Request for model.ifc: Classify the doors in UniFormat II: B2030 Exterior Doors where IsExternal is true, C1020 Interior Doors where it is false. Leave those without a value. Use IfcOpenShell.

First a look at what the model holds.

```python
import ifcopenshell
import ifcopenshell.util.element

model = ifcopenshell.open("model.ifc")
print(model.schema)
print("classifications:", [c.Name for c in model.by_type("IfcClassification")])
values = [ifcopenshell.util.element.get_pset(e, "Pset_DoorCommon", "IsExternal") for e in model.by_type("IfcDoor")]
for value in (True, False, None):
    print("IsExternal", value, values.count(value))
```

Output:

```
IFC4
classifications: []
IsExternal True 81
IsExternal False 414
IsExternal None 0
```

```python
import ifcopenshell
import ifcopenshell.api.classification
import ifcopenshell.util.element

model = ifcopenshell.open("model.ifc")

system = ifcopenshell.api.classification.add_classification(model, classification="UniFormat II")

doors = model.by_type("IfcDoor")
external = {e: ifcopenshell.util.element.get_pset(e, "Pset_DoorCommon", "IsExternal") for e in doors}
for flag, code, name in ((True, "B2030", "Exterior Doors"), (False, "C1020", "Interior Doors")):
    products = [e for e in doors if external[e] is flag]
    ifcopenshell.api.classification.add_reference(
        model, products=products, classification=system, identification=code, name=name
    )
    print(code, len(products))

model.write("model_v2.ifc")
```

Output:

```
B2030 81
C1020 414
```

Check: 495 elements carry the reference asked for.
